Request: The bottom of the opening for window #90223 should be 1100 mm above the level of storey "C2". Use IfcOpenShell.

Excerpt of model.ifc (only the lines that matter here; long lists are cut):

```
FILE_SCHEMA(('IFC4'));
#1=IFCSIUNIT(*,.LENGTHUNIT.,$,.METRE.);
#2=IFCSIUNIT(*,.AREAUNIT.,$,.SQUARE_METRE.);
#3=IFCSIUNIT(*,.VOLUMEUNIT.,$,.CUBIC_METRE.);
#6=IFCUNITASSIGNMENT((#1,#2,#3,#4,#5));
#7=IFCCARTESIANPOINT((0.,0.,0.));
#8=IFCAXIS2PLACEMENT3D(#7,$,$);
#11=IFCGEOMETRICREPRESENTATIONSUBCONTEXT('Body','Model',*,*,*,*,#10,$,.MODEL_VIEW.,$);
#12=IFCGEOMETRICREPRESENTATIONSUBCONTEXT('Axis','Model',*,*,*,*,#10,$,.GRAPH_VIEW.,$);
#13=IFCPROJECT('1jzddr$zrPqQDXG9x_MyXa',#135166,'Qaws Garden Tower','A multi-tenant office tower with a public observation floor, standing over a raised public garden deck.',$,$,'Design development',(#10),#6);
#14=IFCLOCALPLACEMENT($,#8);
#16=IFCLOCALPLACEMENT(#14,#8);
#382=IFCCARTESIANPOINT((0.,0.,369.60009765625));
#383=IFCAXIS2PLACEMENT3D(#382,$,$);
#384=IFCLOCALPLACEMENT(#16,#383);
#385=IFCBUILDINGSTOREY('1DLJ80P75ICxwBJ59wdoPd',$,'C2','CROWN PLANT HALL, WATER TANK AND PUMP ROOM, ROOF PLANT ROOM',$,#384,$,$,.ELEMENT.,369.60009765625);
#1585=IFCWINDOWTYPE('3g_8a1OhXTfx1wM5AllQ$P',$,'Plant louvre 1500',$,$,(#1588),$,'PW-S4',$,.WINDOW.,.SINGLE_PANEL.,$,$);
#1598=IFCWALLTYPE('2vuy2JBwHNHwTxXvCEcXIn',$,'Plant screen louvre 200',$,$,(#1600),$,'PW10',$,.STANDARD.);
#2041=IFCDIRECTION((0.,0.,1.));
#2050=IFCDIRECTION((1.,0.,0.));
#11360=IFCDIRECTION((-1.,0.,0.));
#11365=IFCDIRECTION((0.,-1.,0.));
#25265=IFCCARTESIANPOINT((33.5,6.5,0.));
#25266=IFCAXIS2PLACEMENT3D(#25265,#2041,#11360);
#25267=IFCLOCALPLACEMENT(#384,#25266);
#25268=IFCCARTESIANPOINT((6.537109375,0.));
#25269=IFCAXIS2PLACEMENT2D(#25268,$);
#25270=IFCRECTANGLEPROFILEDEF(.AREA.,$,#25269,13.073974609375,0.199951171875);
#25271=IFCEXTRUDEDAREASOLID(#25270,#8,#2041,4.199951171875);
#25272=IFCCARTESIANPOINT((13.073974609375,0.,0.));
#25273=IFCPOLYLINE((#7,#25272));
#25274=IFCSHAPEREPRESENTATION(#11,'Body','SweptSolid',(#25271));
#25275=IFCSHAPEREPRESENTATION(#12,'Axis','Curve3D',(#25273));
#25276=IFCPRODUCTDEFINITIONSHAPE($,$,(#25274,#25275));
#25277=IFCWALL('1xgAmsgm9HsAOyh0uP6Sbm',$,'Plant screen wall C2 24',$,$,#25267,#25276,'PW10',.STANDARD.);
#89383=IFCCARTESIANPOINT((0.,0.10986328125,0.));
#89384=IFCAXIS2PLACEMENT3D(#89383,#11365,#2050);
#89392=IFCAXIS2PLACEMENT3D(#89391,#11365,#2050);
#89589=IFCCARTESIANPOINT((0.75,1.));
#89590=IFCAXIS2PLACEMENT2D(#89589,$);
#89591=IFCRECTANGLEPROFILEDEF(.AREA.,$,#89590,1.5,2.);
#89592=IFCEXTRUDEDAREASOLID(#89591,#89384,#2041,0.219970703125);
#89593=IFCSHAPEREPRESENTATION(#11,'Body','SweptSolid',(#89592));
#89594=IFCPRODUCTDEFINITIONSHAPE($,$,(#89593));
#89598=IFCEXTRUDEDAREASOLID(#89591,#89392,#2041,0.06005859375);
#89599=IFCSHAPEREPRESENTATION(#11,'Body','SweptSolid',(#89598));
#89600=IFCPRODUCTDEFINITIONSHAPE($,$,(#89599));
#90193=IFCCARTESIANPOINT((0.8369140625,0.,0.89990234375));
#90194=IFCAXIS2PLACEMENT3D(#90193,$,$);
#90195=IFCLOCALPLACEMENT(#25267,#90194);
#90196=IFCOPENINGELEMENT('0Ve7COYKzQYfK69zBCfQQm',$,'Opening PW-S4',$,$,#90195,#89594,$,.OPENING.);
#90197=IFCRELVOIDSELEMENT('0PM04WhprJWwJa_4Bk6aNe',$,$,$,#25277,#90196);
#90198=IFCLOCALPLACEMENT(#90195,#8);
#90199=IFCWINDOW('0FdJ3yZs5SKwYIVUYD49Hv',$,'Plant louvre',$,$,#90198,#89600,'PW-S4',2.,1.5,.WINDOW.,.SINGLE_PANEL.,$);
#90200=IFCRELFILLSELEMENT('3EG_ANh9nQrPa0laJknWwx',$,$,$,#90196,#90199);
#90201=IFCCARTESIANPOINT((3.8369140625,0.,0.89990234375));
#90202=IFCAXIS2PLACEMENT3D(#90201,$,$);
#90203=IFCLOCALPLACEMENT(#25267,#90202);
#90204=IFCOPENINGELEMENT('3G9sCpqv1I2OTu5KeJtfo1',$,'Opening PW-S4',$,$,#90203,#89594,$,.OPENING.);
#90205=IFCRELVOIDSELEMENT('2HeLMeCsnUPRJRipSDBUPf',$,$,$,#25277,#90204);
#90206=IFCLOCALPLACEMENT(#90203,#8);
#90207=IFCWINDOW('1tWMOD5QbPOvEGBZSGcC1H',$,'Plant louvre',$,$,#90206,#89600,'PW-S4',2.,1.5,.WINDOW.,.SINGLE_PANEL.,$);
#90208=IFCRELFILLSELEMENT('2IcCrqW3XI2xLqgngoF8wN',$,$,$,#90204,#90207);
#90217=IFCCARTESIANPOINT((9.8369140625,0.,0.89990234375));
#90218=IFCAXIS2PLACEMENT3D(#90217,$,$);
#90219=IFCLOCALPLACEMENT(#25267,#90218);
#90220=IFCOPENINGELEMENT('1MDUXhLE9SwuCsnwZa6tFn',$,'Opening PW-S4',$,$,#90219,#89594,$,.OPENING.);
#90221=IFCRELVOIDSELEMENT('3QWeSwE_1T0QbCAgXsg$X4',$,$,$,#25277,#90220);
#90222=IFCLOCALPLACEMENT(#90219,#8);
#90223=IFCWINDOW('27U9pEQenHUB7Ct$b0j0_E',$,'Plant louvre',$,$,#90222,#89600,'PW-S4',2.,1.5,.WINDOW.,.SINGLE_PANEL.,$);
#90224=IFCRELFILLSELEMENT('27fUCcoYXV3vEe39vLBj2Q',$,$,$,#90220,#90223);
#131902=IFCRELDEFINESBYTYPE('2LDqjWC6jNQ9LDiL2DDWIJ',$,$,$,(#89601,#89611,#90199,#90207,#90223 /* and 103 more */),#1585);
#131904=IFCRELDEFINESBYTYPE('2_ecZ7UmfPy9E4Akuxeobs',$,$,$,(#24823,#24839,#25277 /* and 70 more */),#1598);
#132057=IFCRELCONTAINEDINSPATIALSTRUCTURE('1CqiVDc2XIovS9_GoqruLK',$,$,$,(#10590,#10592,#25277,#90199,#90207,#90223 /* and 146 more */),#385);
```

```python
import numpy as np
import ifcopenshell
import ifcopenshell.api.geometry
import ifcopenshell.geom
import ifcopenshell.util.element
import ifcopenshell.util.placement
import ifcopenshell.util.shape
import ifcopenshell.util.unit

model = ifcopenshell.open("model.ifc")
unit_scale = ifcopenshell.util.unit.calculate_unit_scale(model)

window = model.by_guid("27U9pEQenHUB7Ct$b0j0_E")
opening = window.FillsVoids[0].RelatingOpeningElement
storey = ifcopenshell.util.element.get_container(window, ifc_class="IfcBuildingStorey")
level = ifcopenshell.util.placement.get_local_placement(storey.ObjectPlacement)[2, 3]

# The opening's origin need not be at the sill, so measure its lowest point.
shape = ifcopenshell.geom.create_shape(ifcopenshell.geom.settings(), opening)
bottom = ifcopenshell.util.shape.get_shape_bottom_elevation(shape, shape.geometry) / unit_scale
dz = level + 1.1 - bottom

shift = np.array([0.0, 0.0, dz])
# The window is placed relative to its opening, so it follows when the opening moves.
matrix = ifcopenshell.util.placement.get_local_placement(opening.ObjectPlacement)
matrix[:3, 3] += shift
ifcopenshell.api.geometry.edit_object_placement(
    model, product=opening, matrix=matrix, is_si=False, should_transform_children=True
)

print(f"moved by {dz * unit_scale:+.3f} m")

model.write("model_v2.ifc")
```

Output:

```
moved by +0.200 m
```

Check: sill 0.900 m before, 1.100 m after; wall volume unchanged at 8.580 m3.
